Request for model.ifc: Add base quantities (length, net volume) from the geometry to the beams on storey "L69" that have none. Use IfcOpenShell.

First a look at what the model holds.

```python
import ifcopenshell
import ifcopenshell.util.element
import ifcopenshell.util.unit

model = ifcopenshell.open("model.ifc")
print(model.schema)
for unit_type in ("LENGTHUNIT", "AREAUNIT", "VOLUMEUNIT"):
    print(unit_type, ifcopenshell.util.unit.calculate_unit_scale(model, unit_type))
storey = next(s for s in model.by_type("IfcBuildingStorey") if s.Name == "L69")
beams = [e for e in ifcopenshell.util.element.get_decomposition(storey) if e.is_a("IfcBeam")]
for e in sorted(beams, key=lambda e: e.id()):
    print(e.id(), e.is_a(), e.Name, list(ifcopenshell.util.element.get_psets(e, qtos_only=True)), sep=" | ")
```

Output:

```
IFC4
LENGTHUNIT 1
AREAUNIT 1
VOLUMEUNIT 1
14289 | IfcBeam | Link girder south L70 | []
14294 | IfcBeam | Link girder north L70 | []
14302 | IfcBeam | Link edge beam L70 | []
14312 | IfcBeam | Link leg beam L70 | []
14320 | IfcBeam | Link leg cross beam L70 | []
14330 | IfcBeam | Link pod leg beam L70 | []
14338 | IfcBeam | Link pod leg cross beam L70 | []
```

```python
import ifcopenshell
import ifcopenshell.api.pset
import ifcopenshell.geom
import ifcopenshell.util.element
import ifcopenshell.util.shape
import ifcopenshell.util.unit

model = ifcopenshell.open("model.ifc")
unit_scale = ifcopenshell.util.unit.calculate_unit_scale(model)
volume_scale = ifcopenshell.util.unit.calculate_unit_scale(model, "VOLUMEUNIT")
settings = ifcopenshell.geom.settings()

storey = next(s for s in model.by_type("IfcBuildingStorey") if s.Name == "L69")
beams = [e for e in ifcopenshell.util.element.get_decomposition(storey) if e.is_a("IfcBeam")]

for e in sorted(beams, key=lambda e: e.id()):
    if ifcopenshell.util.element.get_psets(e, qtos_only=True, should_inherit=False):
        continue
    # Geometry comes back in metres, in the element's own axes.
    shape = ifcopenshell.geom.create_shape(settings, e)
    values = {
        "Length": ifcopenshell.util.shape.get_max_xyz(shape.geometry) / unit_scale,
        "NetVolume": ifcopenshell.util.shape.get_volume(shape.geometry) / volume_scale,
    }
    qto = ifcopenshell.api.pset.add_qto(model, product=e, name="Qto_BeamBaseQuantities")
    ifcopenshell.api.pset.edit_qto(model, qto=qto, properties=values)
    print(e.id(), {k: round(v, 3) for k, v in values.items()})

model.write("model_rev.ifc")
```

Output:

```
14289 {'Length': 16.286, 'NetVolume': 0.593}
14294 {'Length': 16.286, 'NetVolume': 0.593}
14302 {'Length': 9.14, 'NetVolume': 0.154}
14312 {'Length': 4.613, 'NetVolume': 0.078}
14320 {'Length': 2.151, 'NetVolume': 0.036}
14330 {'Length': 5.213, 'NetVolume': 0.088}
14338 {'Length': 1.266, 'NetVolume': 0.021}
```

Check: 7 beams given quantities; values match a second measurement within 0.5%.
